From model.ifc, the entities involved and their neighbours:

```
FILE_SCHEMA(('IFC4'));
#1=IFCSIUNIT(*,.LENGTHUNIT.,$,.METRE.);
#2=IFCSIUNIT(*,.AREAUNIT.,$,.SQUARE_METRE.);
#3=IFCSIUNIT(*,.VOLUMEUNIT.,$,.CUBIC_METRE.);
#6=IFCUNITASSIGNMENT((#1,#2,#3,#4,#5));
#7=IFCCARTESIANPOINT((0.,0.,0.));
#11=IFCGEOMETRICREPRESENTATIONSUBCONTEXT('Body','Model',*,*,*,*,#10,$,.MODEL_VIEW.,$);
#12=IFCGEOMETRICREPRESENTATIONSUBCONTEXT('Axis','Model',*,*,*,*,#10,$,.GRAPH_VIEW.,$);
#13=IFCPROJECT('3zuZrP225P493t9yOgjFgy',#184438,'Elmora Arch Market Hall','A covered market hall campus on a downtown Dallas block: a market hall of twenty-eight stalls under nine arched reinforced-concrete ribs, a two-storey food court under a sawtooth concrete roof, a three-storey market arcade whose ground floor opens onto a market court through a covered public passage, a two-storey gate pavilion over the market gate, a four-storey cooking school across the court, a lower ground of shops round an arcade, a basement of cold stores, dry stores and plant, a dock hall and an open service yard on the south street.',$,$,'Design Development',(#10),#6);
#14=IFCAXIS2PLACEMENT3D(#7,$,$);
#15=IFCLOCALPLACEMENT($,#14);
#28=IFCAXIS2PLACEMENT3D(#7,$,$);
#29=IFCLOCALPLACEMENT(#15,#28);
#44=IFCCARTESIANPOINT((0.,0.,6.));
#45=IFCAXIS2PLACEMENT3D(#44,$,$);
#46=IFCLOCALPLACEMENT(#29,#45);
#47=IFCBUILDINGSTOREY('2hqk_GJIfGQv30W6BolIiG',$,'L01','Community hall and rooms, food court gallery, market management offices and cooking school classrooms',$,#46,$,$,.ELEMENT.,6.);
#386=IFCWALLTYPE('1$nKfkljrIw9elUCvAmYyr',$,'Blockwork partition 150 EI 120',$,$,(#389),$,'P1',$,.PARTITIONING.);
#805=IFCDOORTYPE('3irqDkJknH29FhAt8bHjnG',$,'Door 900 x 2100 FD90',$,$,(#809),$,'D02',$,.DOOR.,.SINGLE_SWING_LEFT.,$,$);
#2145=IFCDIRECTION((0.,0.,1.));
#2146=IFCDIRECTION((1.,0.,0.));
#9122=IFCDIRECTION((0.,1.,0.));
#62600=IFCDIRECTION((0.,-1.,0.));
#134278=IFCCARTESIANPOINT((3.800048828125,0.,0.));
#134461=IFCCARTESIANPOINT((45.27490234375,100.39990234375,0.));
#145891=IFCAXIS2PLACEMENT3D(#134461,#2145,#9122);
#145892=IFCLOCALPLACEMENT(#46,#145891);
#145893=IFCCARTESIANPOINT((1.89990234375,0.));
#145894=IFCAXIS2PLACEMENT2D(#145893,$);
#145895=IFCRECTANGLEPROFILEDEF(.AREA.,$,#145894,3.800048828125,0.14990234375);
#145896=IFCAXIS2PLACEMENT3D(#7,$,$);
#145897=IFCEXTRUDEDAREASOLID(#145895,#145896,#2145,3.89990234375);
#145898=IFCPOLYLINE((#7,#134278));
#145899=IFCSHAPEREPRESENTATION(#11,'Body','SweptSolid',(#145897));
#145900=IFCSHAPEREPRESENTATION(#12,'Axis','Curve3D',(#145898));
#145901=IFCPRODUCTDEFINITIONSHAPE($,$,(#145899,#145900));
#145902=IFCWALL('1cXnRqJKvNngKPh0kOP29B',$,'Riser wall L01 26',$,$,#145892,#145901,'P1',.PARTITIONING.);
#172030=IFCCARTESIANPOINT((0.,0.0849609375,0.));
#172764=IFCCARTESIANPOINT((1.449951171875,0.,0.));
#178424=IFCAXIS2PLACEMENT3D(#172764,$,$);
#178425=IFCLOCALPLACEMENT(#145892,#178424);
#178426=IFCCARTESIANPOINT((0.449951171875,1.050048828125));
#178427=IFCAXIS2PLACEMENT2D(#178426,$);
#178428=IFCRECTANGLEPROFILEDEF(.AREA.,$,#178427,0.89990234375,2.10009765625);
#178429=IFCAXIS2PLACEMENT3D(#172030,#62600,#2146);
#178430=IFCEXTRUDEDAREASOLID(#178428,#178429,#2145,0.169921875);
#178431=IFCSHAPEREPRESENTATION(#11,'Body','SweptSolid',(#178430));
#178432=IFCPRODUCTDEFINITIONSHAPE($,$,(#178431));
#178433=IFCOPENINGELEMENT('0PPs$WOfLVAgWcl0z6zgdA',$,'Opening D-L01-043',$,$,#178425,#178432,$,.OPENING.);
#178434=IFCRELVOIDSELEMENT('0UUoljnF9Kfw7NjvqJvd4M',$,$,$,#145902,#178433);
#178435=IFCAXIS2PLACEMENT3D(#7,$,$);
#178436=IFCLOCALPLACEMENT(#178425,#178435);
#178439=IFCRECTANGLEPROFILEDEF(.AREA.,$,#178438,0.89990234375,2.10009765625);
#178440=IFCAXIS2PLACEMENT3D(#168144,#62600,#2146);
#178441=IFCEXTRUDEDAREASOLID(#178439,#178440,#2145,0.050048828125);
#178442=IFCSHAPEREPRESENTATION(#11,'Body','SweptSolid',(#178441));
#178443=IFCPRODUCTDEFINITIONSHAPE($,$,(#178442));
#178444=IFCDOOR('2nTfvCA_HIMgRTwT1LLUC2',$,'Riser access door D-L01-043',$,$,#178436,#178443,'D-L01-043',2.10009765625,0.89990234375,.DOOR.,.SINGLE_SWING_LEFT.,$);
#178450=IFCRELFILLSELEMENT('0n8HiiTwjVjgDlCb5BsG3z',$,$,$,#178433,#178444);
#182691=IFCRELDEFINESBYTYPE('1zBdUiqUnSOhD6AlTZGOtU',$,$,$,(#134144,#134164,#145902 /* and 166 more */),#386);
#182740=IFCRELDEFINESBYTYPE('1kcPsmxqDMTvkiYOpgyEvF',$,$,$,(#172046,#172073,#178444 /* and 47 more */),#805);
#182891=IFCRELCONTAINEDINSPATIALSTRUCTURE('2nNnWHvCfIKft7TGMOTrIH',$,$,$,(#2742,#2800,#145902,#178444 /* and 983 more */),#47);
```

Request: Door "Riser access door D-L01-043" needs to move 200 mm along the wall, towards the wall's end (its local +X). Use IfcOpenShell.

```python
import ifcopenshell
import ifcopenshell.api.geometry
import ifcopenshell.util.placement

model = ifcopenshell.open("model.ifc")

door = model.by_guid("2nTfvCA_HIMgRTwT1LLUC2")
opening = door.FillsVoids[0].RelatingOpeningElement
wall = opening.VoidsElements[0].RelatingBuildingElement

wall_matrix = ifcopenshell.util.placement.get_local_placement(wall.ObjectPlacement)
shift = wall_matrix[:3, 0] * 0.2
before = ifcopenshell.util.placement.get_local_placement(door.ObjectPlacement)[:3, 3].copy()

# The door is placed relative to its opening, so it follows when the opening moves.
matrix = ifcopenshell.util.placement.get_local_placement(opening.ObjectPlacement)
matrix[:3, 3] += shift
ifcopenshell.api.geometry.edit_object_placement(
    model, product=opening, matrix=matrix, is_si=False, should_transform_children=True
)

after = ifcopenshell.util.placement.get_local_placement(door.ObjectPlacement)[:3, 3]
print("door moved by", (after - before).round(3) + 0.0)

model.write("model_rev.ifc")
```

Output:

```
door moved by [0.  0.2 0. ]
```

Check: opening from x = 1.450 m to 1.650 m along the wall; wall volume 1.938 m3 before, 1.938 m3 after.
